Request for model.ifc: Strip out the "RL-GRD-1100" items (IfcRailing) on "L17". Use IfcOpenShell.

First a look at what the model holds.

```python
import ifcopenshell
import ifcopenshell.util.element

model = ifcopenshell.open("model.ifc")
print(model.schema)
storey = next(s for s in model.by_type("IfcBuildingStorey") if s.Name == "L17")
railings = [e for e in ifcopenshell.util.element.get_decomposition(storey) if e.is_a("IfcRailing")]
seen = {}
for e in railings:
    element_type = ifcopenshell.util.element.get_type(e)
    name = element_type.Name if element_type not in (None, e) else None
    seen[name] = seen.get(name, 0) + 1
for name, count in sorted(seen.items(), key=str):
    print(count, "x", name)
```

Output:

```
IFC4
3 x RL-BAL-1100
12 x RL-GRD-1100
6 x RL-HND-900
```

```python
import ifcopenshell
import ifcopenshell.api.root
import ifcopenshell.util.element

model = ifcopenshell.open("model.ifc")

storey = next(s for s in model.by_type("IfcBuildingStorey") if s.Name == "L17")
railings = [e for e in ifcopenshell.util.element.get_decomposition(storey) if e.is_a("IfcRailing")]
targets = [e for e in railings if (t := ifcopenshell.util.element.get_type(e)) not in (None, e) and t.Name == "RL-GRD-1100"]

for e in targets:
    ifcopenshell.api.root.remove_product(model, product=e)
print(len(targets), "removed")

model.write("model_updated.ifc")
```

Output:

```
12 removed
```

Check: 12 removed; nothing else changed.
